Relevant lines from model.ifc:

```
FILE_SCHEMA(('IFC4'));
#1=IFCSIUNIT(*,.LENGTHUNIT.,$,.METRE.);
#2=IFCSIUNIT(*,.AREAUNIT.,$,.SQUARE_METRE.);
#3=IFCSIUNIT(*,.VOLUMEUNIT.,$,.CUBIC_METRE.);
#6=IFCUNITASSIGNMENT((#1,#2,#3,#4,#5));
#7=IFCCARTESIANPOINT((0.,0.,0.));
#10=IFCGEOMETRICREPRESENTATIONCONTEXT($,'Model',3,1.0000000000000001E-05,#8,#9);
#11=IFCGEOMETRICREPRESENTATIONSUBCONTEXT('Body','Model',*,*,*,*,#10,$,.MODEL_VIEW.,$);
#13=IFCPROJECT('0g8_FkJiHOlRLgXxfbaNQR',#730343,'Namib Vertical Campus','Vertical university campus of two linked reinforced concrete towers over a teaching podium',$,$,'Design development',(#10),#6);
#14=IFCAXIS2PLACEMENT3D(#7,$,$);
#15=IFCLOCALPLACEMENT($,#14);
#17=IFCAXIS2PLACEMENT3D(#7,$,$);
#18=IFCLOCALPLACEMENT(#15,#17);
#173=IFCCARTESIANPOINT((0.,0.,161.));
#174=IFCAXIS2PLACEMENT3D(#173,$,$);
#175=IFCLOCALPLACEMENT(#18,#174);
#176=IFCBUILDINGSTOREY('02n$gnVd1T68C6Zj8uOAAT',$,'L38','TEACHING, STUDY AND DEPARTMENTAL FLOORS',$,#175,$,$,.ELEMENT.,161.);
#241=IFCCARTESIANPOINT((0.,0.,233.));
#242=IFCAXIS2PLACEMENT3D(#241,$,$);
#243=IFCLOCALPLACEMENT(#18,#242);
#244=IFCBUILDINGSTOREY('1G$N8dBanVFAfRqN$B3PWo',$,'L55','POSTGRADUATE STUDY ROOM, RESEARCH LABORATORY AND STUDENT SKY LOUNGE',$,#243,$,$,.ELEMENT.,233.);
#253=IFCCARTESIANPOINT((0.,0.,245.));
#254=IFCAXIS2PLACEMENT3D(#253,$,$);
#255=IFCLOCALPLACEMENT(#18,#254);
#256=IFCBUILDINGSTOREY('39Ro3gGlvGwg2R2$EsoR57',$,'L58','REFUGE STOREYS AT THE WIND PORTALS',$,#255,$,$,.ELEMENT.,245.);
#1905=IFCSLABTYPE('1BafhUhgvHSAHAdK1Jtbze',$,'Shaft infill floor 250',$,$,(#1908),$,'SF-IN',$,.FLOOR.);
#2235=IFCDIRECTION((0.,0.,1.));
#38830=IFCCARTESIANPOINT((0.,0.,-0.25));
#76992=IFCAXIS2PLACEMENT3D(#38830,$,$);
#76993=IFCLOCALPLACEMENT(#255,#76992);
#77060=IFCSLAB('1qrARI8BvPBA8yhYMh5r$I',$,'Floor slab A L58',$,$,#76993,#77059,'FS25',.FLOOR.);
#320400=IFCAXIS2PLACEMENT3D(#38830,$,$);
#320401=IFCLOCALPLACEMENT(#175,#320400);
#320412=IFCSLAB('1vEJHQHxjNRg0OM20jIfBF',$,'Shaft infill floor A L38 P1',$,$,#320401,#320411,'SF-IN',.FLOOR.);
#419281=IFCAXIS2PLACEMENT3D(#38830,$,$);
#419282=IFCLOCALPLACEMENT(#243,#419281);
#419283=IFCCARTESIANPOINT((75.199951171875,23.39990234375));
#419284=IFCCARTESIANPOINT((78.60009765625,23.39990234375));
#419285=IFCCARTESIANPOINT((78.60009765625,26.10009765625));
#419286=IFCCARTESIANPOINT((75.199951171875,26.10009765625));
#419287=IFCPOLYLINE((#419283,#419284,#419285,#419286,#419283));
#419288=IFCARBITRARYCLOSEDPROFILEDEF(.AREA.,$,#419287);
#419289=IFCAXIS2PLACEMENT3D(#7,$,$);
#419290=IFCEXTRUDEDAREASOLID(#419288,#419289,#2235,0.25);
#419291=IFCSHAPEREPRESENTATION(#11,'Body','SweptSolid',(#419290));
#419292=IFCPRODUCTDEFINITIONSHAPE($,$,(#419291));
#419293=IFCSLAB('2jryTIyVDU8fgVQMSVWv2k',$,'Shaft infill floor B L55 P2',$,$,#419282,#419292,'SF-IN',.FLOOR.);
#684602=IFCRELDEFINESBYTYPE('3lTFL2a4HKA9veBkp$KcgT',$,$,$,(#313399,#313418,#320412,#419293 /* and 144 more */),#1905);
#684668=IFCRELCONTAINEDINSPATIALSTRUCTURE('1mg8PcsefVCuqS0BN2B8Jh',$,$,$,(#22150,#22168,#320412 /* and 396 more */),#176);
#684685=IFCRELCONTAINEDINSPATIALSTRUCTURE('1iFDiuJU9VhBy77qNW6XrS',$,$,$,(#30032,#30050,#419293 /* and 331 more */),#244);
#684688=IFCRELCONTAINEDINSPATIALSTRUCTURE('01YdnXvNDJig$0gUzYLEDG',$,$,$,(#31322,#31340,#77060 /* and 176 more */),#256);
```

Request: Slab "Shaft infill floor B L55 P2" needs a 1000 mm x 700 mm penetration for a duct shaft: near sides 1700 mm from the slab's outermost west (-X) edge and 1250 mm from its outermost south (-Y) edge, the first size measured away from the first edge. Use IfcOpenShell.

```python
import numpy as np
import ifcopenshell
import ifcopenshell.api.feature
import ifcopenshell.api.geometry
import ifcopenshell.api.root
import ifcopenshell.geom
import ifcopenshell.util.placement
import ifcopenshell.util.representation
import ifcopenshell.util.shape
import ifcopenshell.util.unit

model = ifcopenshell.open("model.ifc")
unit_scale = ifcopenshell.util.unit.calculate_unit_scale(model)
settings = ifcopenshell.geom.settings()


def volume(element):
    """Net volume in cubic metres, openings subtracted."""
    shape = ifcopenshell.geom.create_shape(settings, element)
    return ifcopenshell.util.shape.get_volume(shape.geometry)


slab = model.by_id(419293)
before = volume(slab)

# Extent in the slab's own axes, in metres. The edges named are its -X and -Y sides.
slab_shape = ifcopenshell.geom.create_shape(settings, slab)
vertices = ifcopenshell.util.shape.get_vertices(slab_shape.geometry)
x_min, y_min, bottom = vertices.min(axis=0)
top = vertices[:, 2].max()

opening = ifcopenshell.api.root.create_entity(model, ifc_class="IfcOpeningElement", name="Duct shaft opening", predefined_type="OPENING")
context = ifcopenshell.util.representation.get_context(model, "Model", "Body", "MODEL_VIEW")
width, depth = 1, 0.7
outline = [(0.0, 0.0), (width, 0.0), (width, depth), (0.0, depth), (0.0, 0.0)]
# Overshoot both faces by 50 mm so the cut is clean.
shape = ifcopenshell.api.geometry.add_slab_representation(
    model, context=context, depth=top - bottom + 0.1, polyline=outline
)
ifcopenshell.api.geometry.assign_representation(model, product=opening, representation=shape)

matrix = ifcopenshell.util.placement.get_local_placement(slab.ObjectPlacement)
matrix[:, 3] = matrix @ np.append(np.array([x_min + 1.7, y_min + 1.25, bottom - 0.05]) / unit_scale, 1.0)
ifcopenshell.api.geometry.edit_object_placement(model, product=opening, matrix=matrix, is_si=False)
ifcopenshell.api.feature.add_feature(model, feature=opening, element=slab)

after = volume(slab)

print(f"slab volume {before:.3f} -> {after:.3f} m3")

model.write("model_updated.ifc")
```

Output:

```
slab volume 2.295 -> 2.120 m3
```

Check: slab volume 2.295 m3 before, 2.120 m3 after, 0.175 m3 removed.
